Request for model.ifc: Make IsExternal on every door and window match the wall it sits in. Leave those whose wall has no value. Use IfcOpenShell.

First a look at what the model holds.

```python
import ifcopenshell
import ifcopenshell.util.element

model = ifcopenshell.open("model.ifc")
print(model.schema)
seen = {}
for e in model.by_type("IfcDoor") + model.by_type("IfcWindow"):
    if not e.FillsVoids:
        continue
    host = e.FillsVoids[0].RelatingOpeningElement.VoidsElements[0].RelatingBuildingElement
    own = ifcopenshell.util.element.get_pset(e, f"Pset_{e.is_a()[3:].removesuffix('StandardCase')}Common", "IsExternal")
    wall = ifcopenshell.util.element.get_pset(host, "Pset_WallCommon", "IsExternal")
    seen[e.is_a(), own, wall] = seen.get((e.is_a(), own, wall), 0) + 1
for (cls, own, wall), count in sorted(seen.items(), key=str):
    print(count, cls, "IsExternal:", own, "| host wall:", wall)
```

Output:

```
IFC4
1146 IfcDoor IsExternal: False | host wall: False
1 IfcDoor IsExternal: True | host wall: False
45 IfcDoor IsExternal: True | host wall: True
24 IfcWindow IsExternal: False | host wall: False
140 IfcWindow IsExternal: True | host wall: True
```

```python
import ifcopenshell
import ifcopenshell.api.pset
import ifcopenshell.util.element

model = ifcopenshell.open("model.ifc")

count = 0
for ifc_class, pset_name in (("IfcDoor", "Pset_DoorCommon"), ("IfcWindow", "Pset_WindowCommon")):
    for e in model.by_type(ifc_class):
        if not e.FillsVoids:
            continue
        host = e.FillsVoids[0].RelatingOpeningElement.VoidsElements[0].RelatingBuildingElement
        external = ifcopenshell.util.element.get_pset(host, "Pset_WallCommon", "IsExternal")
        if external is None or ifcopenshell.util.element.get_pset(e, pset_name, "IsExternal") == external:
            continue
        pset = ifcopenshell.api.pset.add_pset(model, product=e, name=pset_name)
        ifcopenshell.api.pset.edit_pset(model, pset=pset, properties={"IsExternal": external})
        count += 1

print(count, "updated")

model.write("model_updated.ifc")
```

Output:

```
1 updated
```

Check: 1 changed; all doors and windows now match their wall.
